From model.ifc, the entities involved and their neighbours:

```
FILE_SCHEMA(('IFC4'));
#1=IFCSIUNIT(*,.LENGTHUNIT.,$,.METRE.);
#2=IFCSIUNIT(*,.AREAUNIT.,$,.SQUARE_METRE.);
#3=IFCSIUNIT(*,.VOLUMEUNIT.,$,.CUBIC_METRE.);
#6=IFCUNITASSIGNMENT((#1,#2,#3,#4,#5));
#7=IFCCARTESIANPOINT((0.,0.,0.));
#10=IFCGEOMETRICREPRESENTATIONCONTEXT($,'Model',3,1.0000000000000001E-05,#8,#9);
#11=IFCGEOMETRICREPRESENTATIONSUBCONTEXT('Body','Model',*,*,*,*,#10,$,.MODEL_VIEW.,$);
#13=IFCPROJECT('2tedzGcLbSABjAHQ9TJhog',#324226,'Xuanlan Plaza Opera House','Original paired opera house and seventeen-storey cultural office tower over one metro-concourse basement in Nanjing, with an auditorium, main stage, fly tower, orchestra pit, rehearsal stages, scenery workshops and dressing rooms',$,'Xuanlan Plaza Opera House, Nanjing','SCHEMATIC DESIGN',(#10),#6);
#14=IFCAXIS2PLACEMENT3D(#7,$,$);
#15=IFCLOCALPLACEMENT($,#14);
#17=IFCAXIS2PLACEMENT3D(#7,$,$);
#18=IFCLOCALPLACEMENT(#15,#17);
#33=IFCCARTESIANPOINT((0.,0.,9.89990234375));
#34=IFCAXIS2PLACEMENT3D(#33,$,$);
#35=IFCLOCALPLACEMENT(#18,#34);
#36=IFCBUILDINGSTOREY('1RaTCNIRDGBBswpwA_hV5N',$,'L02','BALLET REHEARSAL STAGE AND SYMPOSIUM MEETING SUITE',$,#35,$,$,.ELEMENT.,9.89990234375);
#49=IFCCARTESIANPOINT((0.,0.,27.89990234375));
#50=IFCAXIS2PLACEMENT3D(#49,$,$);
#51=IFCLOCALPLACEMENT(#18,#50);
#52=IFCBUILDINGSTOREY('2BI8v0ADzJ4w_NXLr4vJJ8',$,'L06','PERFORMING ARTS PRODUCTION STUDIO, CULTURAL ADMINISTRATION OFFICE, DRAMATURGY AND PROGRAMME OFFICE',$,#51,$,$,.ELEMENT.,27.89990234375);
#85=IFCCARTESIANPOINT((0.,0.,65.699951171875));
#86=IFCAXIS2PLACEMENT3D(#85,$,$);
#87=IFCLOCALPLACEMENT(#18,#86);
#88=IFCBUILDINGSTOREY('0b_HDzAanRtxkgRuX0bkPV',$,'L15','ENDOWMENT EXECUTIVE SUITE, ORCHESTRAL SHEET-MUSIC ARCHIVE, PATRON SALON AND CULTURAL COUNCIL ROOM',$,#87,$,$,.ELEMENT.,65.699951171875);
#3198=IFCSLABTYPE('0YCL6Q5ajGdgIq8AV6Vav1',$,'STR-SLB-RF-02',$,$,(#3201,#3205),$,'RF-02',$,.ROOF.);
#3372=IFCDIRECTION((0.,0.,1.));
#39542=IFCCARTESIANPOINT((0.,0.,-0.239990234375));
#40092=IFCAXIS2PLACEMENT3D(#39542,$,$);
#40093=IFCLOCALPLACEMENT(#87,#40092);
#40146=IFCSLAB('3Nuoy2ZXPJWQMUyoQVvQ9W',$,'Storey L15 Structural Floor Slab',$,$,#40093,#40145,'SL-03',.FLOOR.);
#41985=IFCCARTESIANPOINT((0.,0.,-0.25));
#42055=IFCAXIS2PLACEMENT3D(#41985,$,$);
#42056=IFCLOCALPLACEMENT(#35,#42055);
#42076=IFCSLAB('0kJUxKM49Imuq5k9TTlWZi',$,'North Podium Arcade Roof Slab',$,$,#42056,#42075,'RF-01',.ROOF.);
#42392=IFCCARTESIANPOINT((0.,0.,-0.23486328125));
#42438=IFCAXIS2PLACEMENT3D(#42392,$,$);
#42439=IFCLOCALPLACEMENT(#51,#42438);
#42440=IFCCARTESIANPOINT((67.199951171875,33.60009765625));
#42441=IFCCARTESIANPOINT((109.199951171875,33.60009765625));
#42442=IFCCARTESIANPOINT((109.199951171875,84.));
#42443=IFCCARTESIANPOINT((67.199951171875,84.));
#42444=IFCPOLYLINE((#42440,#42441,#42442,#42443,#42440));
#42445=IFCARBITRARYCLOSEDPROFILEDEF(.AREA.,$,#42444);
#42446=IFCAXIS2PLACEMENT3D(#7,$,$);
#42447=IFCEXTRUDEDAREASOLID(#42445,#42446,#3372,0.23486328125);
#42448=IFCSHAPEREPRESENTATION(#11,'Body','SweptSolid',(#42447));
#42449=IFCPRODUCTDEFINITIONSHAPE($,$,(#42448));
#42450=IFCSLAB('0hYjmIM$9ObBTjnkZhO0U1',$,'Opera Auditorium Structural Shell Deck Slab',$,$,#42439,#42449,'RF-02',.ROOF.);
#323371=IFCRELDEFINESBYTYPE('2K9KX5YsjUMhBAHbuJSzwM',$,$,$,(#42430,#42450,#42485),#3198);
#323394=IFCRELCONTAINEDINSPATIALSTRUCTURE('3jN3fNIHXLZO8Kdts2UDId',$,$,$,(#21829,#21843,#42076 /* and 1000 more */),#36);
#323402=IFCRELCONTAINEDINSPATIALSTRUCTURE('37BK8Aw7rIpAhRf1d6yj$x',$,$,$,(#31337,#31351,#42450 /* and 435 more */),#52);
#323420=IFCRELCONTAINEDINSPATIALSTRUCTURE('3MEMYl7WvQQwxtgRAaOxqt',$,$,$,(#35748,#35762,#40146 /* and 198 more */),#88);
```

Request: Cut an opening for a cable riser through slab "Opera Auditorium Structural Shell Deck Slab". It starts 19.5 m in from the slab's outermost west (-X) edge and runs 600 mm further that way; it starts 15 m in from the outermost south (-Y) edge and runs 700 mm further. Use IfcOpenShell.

```python
import numpy as np
import ifcopenshell
import ifcopenshell.api.feature
import ifcopenshell.api.geometry
import ifcopenshell.api.root
import ifcopenshell.geom
import ifcopenshell.util.placement
import ifcopenshell.util.representation
import ifcopenshell.util.shape
import ifcopenshell.util.unit

model = ifcopenshell.open("model.ifc")
unit_scale = ifcopenshell.util.unit.calculate_unit_scale(model)
settings = ifcopenshell.geom.settings()


def volume(element):
    """Net volume in cubic metres, openings subtracted."""
    shape = ifcopenshell.geom.create_shape(settings, element)
    return ifcopenshell.util.shape.get_volume(shape.geometry)


slab = model.by_id(42450)
before = volume(slab)

# Extent in the slab's own axes, in metres. The edges named are its -X and -Y sides.
slab_shape = ifcopenshell.geom.create_shape(settings, slab)
vertices = ifcopenshell.util.shape.get_vertices(slab_shape.geometry)
x_min, y_min, bottom = vertices.min(axis=0)
top = vertices[:, 2].max()

opening = ifcopenshell.api.root.create_entity(model, ifc_class="IfcOpeningElement", name="Cable riser opening", predefined_type="OPENING")
context = ifcopenshell.util.representation.get_context(model, "Model", "Body", "MODEL_VIEW")
width, depth = 0.6, 0.7
outline = [(0.0, 0.0), (width, 0.0), (width, depth), (0.0, depth), (0.0, 0.0)]
# Overshoot both faces by 50 mm so the cut is clean.
shape = ifcopenshell.api.geometry.add_slab_representation(
    model, context=context, depth=top - bottom + 0.1, polyline=outline
)
ifcopenshell.api.geometry.assign_representation(model, product=opening, representation=shape)

matrix = ifcopenshell.util.placement.get_local_placement(slab.ObjectPlacement)
matrix[:, 3] = matrix @ np.append(np.array([x_min + 19.5, y_min + 15, bottom - 0.05]) / unit_scale, 1.0)
ifcopenshell.api.geometry.edit_object_placement(model, product=opening, matrix=matrix, is_si=False)
ifcopenshell.api.feature.add_feature(model, feature=opening, element=slab)

after = volume(slab)

print(f"slab volume {before:.3f} -> {after:.3f} m3")

model.write("model_v2.ifc")
```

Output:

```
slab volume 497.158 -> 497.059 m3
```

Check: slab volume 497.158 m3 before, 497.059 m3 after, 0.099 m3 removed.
